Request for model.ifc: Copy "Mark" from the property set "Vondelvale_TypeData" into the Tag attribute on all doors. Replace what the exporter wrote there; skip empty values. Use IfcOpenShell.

First a look at what the model holds.

```python
import ifcopenshell
import ifcopenshell.util.element

model = ifcopenshell.open("model.ifc")
print(model.schema)
doors = model.by_type("IfcDoor")
print(len(doors), "doors")
for e in doors[:8]:
    source = ifcopenshell.util.element.get_pset(e, "Vondelvale_TypeData", "Mark")
    target = e.Tag
    print(e.id(), repr(source), repr(target), sep=" | ")
```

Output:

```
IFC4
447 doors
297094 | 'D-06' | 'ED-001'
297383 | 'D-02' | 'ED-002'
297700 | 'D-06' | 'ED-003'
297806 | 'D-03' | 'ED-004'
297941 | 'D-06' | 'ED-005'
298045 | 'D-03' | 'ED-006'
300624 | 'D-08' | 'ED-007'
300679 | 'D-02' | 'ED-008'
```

```python
import ifcopenshell
import ifcopenshell.util.element

model = ifcopenshell.open("model.ifc")

count = 0
for e in model.by_type("IfcDoor"):
    value = ifcopenshell.util.element.get_pset(e, "Vondelvale_TypeData", "Mark")
    current = e.Tag
    if not value or not value.strip() or current == value:
        continue
    e.Tag = value
    count += 1

print(count, "doors updated")

model.write("model_updated.ifc")
```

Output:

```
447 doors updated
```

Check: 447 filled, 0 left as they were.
